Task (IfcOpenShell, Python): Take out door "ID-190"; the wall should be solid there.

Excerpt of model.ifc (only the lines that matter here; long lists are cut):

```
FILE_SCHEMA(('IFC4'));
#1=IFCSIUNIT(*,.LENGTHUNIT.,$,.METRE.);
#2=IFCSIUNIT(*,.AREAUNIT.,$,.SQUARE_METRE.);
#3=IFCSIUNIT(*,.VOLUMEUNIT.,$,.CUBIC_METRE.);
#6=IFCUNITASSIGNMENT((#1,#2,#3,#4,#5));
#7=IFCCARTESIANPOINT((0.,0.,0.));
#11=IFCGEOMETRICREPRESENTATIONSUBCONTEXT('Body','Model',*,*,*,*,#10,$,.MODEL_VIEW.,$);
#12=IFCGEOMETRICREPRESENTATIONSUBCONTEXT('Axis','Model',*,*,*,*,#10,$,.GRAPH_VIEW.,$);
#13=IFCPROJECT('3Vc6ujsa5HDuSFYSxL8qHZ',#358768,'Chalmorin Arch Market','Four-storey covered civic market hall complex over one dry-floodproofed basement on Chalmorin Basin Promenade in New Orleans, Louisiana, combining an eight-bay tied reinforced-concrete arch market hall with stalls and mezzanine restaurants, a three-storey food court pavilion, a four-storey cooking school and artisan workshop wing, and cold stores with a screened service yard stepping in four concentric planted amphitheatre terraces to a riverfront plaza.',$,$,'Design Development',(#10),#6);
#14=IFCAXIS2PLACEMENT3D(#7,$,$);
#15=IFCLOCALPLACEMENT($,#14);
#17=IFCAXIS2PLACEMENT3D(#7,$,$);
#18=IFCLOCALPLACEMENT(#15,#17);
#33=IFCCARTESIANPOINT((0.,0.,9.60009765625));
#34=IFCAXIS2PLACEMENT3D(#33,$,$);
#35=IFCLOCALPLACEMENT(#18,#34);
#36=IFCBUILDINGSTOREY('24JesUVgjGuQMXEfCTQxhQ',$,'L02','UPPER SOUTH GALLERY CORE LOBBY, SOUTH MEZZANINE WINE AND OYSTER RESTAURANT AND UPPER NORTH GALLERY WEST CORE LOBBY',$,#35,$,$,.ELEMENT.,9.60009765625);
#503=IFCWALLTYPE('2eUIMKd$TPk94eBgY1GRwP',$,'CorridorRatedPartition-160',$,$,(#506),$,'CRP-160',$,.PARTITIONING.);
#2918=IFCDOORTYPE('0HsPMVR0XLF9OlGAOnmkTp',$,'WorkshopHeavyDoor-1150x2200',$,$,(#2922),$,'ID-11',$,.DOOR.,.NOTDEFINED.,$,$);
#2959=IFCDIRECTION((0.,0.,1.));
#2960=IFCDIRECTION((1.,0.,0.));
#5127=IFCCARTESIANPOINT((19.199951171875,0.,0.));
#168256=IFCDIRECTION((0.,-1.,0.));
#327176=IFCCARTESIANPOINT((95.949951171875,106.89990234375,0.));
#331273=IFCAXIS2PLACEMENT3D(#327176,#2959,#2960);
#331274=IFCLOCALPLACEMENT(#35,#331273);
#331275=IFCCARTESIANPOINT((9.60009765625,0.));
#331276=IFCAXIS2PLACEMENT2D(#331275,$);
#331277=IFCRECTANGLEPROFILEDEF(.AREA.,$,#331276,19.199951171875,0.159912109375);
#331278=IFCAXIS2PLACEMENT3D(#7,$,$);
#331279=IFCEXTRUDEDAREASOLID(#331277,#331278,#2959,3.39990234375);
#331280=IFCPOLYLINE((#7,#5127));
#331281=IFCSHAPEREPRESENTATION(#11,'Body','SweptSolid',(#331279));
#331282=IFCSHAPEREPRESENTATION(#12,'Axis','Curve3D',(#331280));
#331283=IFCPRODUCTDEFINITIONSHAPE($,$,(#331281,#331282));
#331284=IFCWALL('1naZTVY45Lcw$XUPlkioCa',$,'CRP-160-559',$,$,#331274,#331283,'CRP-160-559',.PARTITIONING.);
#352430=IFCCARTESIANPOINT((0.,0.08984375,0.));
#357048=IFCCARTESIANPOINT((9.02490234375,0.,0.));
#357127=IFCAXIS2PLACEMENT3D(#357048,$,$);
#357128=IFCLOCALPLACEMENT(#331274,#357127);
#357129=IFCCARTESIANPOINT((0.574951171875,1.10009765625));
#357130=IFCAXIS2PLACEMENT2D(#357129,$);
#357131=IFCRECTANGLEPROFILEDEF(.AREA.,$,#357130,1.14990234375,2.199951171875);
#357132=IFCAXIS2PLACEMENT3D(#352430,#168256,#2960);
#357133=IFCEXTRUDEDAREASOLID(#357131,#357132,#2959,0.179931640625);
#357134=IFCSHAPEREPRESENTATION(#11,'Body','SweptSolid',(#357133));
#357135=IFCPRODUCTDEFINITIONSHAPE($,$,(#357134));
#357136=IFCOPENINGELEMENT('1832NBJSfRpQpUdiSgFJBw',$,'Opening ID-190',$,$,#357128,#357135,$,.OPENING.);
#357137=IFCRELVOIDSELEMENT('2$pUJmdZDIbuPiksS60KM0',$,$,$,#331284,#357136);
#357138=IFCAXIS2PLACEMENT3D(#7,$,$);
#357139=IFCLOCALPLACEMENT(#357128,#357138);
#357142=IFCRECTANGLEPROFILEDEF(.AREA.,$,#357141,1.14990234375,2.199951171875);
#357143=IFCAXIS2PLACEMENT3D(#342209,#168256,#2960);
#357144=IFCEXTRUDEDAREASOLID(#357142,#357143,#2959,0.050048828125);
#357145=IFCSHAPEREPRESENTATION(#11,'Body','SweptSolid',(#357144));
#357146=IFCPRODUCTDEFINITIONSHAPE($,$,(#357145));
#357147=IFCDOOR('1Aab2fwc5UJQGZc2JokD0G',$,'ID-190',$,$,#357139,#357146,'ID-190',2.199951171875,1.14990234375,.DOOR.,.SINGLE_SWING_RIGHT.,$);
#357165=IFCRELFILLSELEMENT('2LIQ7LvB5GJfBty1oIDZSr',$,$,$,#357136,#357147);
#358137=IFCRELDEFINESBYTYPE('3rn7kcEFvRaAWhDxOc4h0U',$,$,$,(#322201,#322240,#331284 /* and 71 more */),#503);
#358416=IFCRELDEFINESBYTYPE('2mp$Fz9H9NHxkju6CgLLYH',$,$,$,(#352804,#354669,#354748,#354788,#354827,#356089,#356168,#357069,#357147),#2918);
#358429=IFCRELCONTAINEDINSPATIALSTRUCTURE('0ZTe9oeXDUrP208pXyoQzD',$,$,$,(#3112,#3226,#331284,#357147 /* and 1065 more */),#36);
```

```python
import ifcopenshell
import ifcopenshell.api.feature
import ifcopenshell.api.root
import ifcopenshell.geom
import ifcopenshell.util.shape

model = ifcopenshell.open("model.ifc")
settings = ifcopenshell.geom.settings()


def volume(element):
    """Net volume in cubic metres, openings subtracted."""
    shape = ifcopenshell.geom.create_shape(settings, element)
    return ifcopenshell.util.shape.get_volume(shape.geometry)


door = model.by_guid("1Aab2fwc5UJQGZc2JokD0G")
opening = door.FillsVoids[0].RelatingOpeningElement
wall = opening.VoidsElements[0].RelatingBuildingElement
before = volume(wall)

ifcopenshell.api.root.remove_product(model, product=door)
ifcopenshell.api.feature.remove_feature(model, feature=opening)

after = volume(wall)

print(f"wall volume {before:.3f} -> {after:.3f} m3")

model.write("model_v2.ifc")
```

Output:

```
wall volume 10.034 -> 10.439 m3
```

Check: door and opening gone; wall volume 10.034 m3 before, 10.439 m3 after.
